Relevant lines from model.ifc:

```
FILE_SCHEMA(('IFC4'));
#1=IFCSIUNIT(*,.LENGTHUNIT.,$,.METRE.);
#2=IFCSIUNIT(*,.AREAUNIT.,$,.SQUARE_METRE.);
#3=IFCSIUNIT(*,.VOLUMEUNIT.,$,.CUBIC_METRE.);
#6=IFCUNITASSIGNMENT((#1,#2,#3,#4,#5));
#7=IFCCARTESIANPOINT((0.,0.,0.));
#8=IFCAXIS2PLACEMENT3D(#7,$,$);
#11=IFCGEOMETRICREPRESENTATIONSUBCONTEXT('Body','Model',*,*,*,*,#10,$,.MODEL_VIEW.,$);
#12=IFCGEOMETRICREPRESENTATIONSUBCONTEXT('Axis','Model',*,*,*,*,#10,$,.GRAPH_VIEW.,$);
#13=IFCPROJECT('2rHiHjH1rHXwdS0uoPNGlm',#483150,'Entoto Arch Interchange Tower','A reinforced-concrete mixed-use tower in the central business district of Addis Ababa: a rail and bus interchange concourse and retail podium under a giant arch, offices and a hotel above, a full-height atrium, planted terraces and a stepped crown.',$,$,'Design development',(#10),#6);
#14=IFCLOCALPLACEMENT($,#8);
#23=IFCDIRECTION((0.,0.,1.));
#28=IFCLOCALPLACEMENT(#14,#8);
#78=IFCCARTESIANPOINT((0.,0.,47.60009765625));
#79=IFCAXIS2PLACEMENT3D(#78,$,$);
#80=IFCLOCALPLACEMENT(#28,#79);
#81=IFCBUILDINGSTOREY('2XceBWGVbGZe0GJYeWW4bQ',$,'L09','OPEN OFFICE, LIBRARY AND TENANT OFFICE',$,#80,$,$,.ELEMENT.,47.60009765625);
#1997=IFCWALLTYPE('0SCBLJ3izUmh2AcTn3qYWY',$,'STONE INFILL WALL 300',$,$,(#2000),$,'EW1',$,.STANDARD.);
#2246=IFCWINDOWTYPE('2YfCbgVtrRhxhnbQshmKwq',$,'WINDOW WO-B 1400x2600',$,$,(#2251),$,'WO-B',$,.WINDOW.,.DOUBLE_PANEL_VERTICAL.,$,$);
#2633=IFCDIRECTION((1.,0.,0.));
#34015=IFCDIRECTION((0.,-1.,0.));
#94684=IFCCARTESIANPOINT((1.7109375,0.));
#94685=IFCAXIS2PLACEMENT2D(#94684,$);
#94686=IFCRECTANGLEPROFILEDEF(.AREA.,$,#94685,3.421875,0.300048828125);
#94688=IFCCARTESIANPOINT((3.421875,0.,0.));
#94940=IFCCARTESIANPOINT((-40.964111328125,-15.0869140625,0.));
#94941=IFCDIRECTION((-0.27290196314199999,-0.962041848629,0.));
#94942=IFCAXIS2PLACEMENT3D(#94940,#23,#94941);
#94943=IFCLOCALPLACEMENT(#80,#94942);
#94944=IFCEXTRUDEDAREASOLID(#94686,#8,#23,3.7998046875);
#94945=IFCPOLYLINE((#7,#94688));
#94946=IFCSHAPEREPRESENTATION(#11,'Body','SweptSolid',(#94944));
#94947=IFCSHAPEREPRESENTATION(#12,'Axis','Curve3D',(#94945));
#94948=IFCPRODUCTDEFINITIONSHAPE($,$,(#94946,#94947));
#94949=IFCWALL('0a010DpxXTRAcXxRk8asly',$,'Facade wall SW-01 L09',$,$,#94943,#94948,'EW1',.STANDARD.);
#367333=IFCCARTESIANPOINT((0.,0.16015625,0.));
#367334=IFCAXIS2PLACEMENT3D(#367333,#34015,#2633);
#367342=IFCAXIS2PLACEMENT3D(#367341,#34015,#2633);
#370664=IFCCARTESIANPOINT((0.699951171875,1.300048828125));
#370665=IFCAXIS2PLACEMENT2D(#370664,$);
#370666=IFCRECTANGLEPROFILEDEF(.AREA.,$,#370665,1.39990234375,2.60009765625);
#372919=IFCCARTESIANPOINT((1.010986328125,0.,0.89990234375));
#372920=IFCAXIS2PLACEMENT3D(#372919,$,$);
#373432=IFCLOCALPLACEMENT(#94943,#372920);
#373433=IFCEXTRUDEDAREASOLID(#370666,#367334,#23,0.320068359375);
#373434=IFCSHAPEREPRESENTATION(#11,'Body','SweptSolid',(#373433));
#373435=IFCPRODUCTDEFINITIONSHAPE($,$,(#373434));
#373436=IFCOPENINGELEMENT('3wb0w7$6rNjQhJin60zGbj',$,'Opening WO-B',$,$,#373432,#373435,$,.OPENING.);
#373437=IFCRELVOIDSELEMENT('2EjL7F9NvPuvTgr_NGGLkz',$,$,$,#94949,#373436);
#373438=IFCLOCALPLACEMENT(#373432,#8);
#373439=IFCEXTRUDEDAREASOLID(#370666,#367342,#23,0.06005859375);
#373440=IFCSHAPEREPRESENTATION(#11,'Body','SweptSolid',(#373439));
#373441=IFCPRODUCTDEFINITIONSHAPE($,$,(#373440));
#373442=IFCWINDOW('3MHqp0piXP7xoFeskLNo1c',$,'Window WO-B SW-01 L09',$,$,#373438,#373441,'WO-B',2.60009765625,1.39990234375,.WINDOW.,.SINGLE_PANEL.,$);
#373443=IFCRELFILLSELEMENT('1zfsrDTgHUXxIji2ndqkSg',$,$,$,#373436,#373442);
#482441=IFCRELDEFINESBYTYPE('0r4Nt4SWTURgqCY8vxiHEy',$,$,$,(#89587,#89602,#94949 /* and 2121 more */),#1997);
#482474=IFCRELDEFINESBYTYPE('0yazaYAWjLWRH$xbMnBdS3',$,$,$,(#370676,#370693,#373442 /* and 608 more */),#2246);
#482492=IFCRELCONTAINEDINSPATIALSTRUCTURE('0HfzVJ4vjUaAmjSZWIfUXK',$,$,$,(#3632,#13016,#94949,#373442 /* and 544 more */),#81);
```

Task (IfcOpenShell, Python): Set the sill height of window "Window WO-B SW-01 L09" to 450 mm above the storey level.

```python
import numpy as np
import ifcopenshell
import ifcopenshell.api.geometry
import ifcopenshell.geom
import ifcopenshell.util.element
import ifcopenshell.util.placement
import ifcopenshell.util.shape
import ifcopenshell.util.unit

model = ifcopenshell.open("model.ifc")
unit_scale = ifcopenshell.util.unit.calculate_unit_scale(model)

window = model.by_id(373442)
opening = window.FillsVoids[0].RelatingOpeningElement
storey = ifcopenshell.util.element.get_container(window, ifc_class="IfcBuildingStorey")
level = ifcopenshell.util.placement.get_local_placement(storey.ObjectPlacement)[2, 3]

# The opening's origin need not be at the sill, so measure its lowest point.
shape = ifcopenshell.geom.create_shape(ifcopenshell.geom.settings(), opening)
bottom = ifcopenshell.util.shape.get_shape_bottom_elevation(shape, shape.geometry) / unit_scale
dz = level + 0.45 / unit_scale - bottom

shift = np.array([0.0, 0.0, dz])
# The window is placed relative to its opening, so it follows when the opening moves.
matrix = ifcopenshell.util.placement.get_local_placement(opening.ObjectPlacement)
matrix[:3, 3] += shift
ifcopenshell.api.geometry.edit_object_placement(
    model, product=opening, matrix=matrix, is_si=False, should_transform_children=True
)

print(f"moved by {dz * unit_scale:+.3f} m")

model.write("model_edited.ifc")
```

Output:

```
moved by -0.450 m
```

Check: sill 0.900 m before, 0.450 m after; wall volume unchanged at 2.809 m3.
